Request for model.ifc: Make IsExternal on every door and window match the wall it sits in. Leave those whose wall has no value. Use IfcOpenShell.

First a look at what the model holds.

```python
import ifcopenshell
import ifcopenshell.util.element

model = ifcopenshell.open("model.ifc")
print(model.schema)
seen = {}
for e in model.by_type("IfcDoor") + model.by_type("IfcWindow"):
    if not e.FillsVoids:
        continue
    host = e.FillsVoids[0].RelatingOpeningElement.VoidsElements[0].RelatingBuildingElement
    own = ifcopenshell.util.element.get_pset(e, f"Pset_{e.is_a()[3:].removesuffix('StandardCase')}Common", "IsExternal")
    wall = ifcopenshell.util.element.get_pset(host, "Pset_WallCommon", "IsExternal")
    seen[e.is_a(), own, wall] = seen.get((e.is_a(), own, wall), 0) + 1
for (cls, own, wall), count in sorted(seen.items(), key=str):
    print(count, cls, "IsExternal:", own, "| host wall:", wall)
```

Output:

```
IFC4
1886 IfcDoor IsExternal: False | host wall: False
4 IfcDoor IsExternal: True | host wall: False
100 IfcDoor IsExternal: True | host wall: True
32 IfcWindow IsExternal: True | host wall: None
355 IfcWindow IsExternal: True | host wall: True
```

```python
import ifcopenshell
import ifcopenshell.api.pset
import ifcopenshell.util.element

model = ifcopenshell.open("model.ifc")

count = 0
for ifc_class, pset_name in (("IfcDoor", "Pset_DoorCommon"), ("IfcWindow", "Pset_WindowCommon")):
    for e in model.by_type(ifc_class):
        if not e.FillsVoids:
            continue
        host = e.FillsVoids[0].RelatingOpeningElement.VoidsElements[0].RelatingBuildingElement
        external = ifcopenshell.util.element.get_pset(host, "Pset_WallCommon", "IsExternal")
        if external is None or ifcopenshell.util.element.get_pset(e, pset_name, "IsExternal") == external:
            continue
        pset = ifcopenshell.api.pset.add_pset(model, product=e, name=pset_name)
        ifcopenshell.api.pset.edit_pset(model, pset=pset, properties={"IsExternal": external})
        count += 1

print(count, "updated")

model.write("model_updated.ifc")
```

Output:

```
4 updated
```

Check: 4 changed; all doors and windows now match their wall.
